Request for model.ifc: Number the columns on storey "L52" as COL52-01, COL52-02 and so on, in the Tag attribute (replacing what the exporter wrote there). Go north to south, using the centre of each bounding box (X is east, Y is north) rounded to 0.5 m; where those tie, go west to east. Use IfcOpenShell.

First a look at what the model holds.

```python
import ifcopenshell
import ifcopenshell.util.element
import ifcopenshell.util.placement

model = ifcopenshell.open("model.ifc")
print(model.schema)
storey = next(s for s in model.by_type("IfcBuildingStorey") if s.Name == "L52")
columns = [e for e in ifcopenshell.util.element.get_decomposition(storey) if e.is_a("IfcColumn")]
for e in sorted(columns, key=lambda e: e.id()):
    origin = ifcopenshell.util.placement.get_local_placement(e.ObjectPlacement)[:3, 3]
    print(e.id(), e.Tag, e.Name, origin.round(2) + 0.0, sep=" | ")
```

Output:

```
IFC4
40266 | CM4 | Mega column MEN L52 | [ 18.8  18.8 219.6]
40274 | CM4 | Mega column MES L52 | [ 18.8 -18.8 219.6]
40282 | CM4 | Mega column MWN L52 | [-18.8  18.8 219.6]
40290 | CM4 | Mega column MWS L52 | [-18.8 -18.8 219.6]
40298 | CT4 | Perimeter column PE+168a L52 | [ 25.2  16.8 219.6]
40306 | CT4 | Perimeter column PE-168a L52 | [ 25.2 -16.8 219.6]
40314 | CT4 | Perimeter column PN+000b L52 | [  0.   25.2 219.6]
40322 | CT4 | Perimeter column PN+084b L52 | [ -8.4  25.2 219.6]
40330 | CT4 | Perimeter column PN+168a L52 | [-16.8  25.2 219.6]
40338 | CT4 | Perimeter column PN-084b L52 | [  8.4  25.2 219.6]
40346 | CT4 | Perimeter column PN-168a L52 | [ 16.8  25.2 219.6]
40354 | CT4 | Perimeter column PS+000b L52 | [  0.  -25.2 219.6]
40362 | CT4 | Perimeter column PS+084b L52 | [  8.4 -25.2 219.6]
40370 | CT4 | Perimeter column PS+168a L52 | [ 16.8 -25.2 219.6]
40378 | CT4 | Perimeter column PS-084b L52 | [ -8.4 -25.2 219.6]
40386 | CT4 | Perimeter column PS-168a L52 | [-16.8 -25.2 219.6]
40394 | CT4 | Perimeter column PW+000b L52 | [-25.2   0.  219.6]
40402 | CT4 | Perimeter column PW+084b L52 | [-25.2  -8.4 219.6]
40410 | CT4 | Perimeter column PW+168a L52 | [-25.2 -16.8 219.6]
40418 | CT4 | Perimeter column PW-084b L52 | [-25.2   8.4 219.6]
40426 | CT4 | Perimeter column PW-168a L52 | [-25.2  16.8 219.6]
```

```python
import ifcopenshell
import ifcopenshell.geom
import ifcopenshell.util.element
import ifcopenshell.util.shape

model = ifcopenshell.open("model.ifc")
settings = ifcopenshell.geom.settings()
settings.set("use-world-coords", True)


def centre(element):
    shape = ifcopenshell.geom.create_shape(settings, element)
    return ifcopenshell.util.shape.get_bbox_centroid(shape.geometry)


storey = next(s for s in model.by_type("IfcBuildingStorey") if s.Name == "L52")
columns = [e for e in ifcopenshell.util.element.get_decomposition(storey) if e.is_a("IfcColumn")]

# Insertion points can sit at a corner or the storey origin, so sort by the geometry (in metres).
centres = {e: centre(e) for e in columns}
columns.sort(key=lambda e: (-round(centres[e][1] / 0.5), centres[e][0]))

for i, e in enumerate(columns, start=1):
    number = f"COL52-{i:02d}"
    e.Tag = number
    print(e.id(), number)

model.write("model_updated.ifc")
```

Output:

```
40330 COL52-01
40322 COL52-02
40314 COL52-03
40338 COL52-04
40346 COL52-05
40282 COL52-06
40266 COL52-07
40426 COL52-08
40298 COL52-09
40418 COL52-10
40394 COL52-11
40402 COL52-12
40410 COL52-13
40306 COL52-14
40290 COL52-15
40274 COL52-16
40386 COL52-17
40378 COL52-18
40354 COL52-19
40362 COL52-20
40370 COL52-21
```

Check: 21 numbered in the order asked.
